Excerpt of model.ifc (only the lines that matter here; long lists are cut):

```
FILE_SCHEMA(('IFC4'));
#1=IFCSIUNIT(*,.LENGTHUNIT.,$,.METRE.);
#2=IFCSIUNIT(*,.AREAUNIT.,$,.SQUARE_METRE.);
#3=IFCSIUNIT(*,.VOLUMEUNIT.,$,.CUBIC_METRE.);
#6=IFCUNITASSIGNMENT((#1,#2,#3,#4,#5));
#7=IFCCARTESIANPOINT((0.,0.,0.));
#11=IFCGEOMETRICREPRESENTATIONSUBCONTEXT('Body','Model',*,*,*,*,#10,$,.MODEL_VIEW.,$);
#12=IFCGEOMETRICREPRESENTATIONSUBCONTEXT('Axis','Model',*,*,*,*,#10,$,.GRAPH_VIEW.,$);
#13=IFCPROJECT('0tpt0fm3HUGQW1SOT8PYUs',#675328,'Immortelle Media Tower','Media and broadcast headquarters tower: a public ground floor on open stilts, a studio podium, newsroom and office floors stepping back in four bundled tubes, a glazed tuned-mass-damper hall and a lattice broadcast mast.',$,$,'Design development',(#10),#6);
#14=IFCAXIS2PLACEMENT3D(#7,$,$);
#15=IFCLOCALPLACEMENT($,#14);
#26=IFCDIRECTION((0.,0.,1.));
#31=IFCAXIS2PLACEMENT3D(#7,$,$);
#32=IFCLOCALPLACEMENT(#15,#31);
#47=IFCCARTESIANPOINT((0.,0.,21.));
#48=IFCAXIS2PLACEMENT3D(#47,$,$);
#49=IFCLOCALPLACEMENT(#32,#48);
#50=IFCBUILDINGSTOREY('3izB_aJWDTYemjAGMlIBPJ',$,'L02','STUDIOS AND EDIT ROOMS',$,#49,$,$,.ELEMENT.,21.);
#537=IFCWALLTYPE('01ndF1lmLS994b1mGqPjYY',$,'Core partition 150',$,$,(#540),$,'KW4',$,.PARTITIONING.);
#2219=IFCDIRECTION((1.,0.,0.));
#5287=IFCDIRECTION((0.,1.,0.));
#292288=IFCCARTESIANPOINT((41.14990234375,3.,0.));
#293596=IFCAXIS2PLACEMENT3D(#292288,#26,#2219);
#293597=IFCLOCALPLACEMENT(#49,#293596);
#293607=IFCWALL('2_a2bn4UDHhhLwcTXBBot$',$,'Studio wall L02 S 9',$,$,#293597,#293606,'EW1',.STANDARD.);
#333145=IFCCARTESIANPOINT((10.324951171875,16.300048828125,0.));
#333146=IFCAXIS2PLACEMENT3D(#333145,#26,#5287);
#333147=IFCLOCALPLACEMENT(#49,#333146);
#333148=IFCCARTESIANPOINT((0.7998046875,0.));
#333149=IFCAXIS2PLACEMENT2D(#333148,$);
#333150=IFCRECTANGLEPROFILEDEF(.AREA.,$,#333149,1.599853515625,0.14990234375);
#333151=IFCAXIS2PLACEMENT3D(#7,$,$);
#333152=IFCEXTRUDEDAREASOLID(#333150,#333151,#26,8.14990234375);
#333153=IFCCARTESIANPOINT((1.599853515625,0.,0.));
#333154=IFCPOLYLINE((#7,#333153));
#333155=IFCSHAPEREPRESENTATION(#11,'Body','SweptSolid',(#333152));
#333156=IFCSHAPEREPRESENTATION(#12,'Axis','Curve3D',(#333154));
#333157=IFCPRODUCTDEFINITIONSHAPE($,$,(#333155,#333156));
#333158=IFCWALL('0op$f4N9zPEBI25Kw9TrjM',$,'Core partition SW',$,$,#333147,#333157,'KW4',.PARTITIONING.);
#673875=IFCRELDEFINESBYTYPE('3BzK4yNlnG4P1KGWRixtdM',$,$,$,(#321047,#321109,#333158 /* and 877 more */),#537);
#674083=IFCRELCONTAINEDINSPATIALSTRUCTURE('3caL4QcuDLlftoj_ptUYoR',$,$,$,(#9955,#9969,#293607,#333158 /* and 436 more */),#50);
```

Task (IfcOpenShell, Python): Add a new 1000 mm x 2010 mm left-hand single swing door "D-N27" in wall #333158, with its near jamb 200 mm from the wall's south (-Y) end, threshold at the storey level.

```python
import numpy as np
import ifcopenshell
import ifcopenshell.api.feature
import ifcopenshell.api.geometry
import ifcopenshell.api.root
import ifcopenshell.api.spatial
import ifcopenshell.geom
import ifcopenshell.util.element
import ifcopenshell.util.placement
import ifcopenshell.util.representation
import ifcopenshell.util.shape
import ifcopenshell.util.unit

model = ifcopenshell.open("model.ifc")
unit_scale = ifcopenshell.util.unit.calculate_unit_scale(model)
settings = ifcopenshell.geom.settings()


def volume(element):
    """Net volume in cubic metres, openings subtracted."""
    shape = ifcopenshell.geom.create_shape(settings, element)
    return ifcopenshell.util.shape.get_volume(shape.geometry)


wall = model.by_id(333158)
storey = ifcopenshell.util.element.get_container(wall, ifc_class="IfcBuildingStorey")
context = ifcopenshell.util.representation.get_context(model, "Model", "Body", "MODEL_VIEW")
before = volume(wall)

width, height, from_end, sill = 1, 2.01, 0.2, 0.0  # metres

# The wall runs along its own X axis, and the end named is its -X end.
wall_shape = ifcopenshell.geom.create_shape(settings, wall)
x, y, z = ifcopenshell.util.shape.get_vertices(wall_shape.geometry).T
start = x.min() + from_end
face, thickness = float(y.min()), float(y.max() - y.min())
wall_matrix = ifcopenshell.util.placement.get_local_placement(wall.ObjectPlacement)
level = ifcopenshell.util.placement.get_local_placement(storey.ObjectPlacement)[2, 3]


def in_wall(x, y):
    """Placement at x, y metres in the wall's axes, at sill height."""
    matrix = wall_matrix.copy()
    matrix[:, 3] = wall_matrix @ np.array([x / unit_scale, y / unit_scale, 0.0, 1.0])
    matrix[2, 3] = level + sill / unit_scale
    return matrix


# Opening: a box that overshoots both wall faces by 50 mm.
opening = ifcopenshell.api.root.create_entity(model, ifc_class="IfcOpeningElement", predefined_type="OPENING")
box = ifcopenshell.api.geometry.add_wall_representation(
    model, context=context, length=width, height=height, thickness=thickness + 0.1
)
ifcopenshell.api.geometry.assign_representation(model, product=opening, representation=box)
ifcopenshell.api.geometry.edit_object_placement(model, product=opening, matrix=in_wall(start, face - 0.05), is_si=False)
ifcopenshell.api.feature.add_feature(model, feature=opening, element=wall)

door = ifcopenshell.api.root.create_entity(model, ifc_class="IfcDoor", name="D-N27", predefined_type="DOOR")
door.OverallWidth, door.OverallHeight = width / unit_scale, height / unit_scale
door.OperationType = "SINGLE_SWING_LEFT"
body = ifcopenshell.api.geometry.add_door_representation(
    model,
    context=context,
    overall_width=door.OverallWidth,
    overall_height=door.OverallHeight,
    operation_type="SINGLE_SWING_LEFT",
    lining_properties={"LiningDepth": thickness / unit_scale, "ThresholdDepth": thickness / unit_scale},
)
ifcopenshell.api.geometry.assign_representation(model, product=door, representation=body)
ifcopenshell.api.spatial.assign_container(model, products=[door], relating_structure=storey)
ifcopenshell.api.feature.add_filling(model, opening=opening, element=door)

# The lining spans the wall, so the door starts at the wall face.
ifcopenshell.api.geometry.edit_object_placement(model, product=door, matrix=in_wall(start, face), is_si=False)

after = volume(wall)

print(f"wall volume {before:.3f} -> {after:.3f} m3")

model.write("model_rev.ifc")
```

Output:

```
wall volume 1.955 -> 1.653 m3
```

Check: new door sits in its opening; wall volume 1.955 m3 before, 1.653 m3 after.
